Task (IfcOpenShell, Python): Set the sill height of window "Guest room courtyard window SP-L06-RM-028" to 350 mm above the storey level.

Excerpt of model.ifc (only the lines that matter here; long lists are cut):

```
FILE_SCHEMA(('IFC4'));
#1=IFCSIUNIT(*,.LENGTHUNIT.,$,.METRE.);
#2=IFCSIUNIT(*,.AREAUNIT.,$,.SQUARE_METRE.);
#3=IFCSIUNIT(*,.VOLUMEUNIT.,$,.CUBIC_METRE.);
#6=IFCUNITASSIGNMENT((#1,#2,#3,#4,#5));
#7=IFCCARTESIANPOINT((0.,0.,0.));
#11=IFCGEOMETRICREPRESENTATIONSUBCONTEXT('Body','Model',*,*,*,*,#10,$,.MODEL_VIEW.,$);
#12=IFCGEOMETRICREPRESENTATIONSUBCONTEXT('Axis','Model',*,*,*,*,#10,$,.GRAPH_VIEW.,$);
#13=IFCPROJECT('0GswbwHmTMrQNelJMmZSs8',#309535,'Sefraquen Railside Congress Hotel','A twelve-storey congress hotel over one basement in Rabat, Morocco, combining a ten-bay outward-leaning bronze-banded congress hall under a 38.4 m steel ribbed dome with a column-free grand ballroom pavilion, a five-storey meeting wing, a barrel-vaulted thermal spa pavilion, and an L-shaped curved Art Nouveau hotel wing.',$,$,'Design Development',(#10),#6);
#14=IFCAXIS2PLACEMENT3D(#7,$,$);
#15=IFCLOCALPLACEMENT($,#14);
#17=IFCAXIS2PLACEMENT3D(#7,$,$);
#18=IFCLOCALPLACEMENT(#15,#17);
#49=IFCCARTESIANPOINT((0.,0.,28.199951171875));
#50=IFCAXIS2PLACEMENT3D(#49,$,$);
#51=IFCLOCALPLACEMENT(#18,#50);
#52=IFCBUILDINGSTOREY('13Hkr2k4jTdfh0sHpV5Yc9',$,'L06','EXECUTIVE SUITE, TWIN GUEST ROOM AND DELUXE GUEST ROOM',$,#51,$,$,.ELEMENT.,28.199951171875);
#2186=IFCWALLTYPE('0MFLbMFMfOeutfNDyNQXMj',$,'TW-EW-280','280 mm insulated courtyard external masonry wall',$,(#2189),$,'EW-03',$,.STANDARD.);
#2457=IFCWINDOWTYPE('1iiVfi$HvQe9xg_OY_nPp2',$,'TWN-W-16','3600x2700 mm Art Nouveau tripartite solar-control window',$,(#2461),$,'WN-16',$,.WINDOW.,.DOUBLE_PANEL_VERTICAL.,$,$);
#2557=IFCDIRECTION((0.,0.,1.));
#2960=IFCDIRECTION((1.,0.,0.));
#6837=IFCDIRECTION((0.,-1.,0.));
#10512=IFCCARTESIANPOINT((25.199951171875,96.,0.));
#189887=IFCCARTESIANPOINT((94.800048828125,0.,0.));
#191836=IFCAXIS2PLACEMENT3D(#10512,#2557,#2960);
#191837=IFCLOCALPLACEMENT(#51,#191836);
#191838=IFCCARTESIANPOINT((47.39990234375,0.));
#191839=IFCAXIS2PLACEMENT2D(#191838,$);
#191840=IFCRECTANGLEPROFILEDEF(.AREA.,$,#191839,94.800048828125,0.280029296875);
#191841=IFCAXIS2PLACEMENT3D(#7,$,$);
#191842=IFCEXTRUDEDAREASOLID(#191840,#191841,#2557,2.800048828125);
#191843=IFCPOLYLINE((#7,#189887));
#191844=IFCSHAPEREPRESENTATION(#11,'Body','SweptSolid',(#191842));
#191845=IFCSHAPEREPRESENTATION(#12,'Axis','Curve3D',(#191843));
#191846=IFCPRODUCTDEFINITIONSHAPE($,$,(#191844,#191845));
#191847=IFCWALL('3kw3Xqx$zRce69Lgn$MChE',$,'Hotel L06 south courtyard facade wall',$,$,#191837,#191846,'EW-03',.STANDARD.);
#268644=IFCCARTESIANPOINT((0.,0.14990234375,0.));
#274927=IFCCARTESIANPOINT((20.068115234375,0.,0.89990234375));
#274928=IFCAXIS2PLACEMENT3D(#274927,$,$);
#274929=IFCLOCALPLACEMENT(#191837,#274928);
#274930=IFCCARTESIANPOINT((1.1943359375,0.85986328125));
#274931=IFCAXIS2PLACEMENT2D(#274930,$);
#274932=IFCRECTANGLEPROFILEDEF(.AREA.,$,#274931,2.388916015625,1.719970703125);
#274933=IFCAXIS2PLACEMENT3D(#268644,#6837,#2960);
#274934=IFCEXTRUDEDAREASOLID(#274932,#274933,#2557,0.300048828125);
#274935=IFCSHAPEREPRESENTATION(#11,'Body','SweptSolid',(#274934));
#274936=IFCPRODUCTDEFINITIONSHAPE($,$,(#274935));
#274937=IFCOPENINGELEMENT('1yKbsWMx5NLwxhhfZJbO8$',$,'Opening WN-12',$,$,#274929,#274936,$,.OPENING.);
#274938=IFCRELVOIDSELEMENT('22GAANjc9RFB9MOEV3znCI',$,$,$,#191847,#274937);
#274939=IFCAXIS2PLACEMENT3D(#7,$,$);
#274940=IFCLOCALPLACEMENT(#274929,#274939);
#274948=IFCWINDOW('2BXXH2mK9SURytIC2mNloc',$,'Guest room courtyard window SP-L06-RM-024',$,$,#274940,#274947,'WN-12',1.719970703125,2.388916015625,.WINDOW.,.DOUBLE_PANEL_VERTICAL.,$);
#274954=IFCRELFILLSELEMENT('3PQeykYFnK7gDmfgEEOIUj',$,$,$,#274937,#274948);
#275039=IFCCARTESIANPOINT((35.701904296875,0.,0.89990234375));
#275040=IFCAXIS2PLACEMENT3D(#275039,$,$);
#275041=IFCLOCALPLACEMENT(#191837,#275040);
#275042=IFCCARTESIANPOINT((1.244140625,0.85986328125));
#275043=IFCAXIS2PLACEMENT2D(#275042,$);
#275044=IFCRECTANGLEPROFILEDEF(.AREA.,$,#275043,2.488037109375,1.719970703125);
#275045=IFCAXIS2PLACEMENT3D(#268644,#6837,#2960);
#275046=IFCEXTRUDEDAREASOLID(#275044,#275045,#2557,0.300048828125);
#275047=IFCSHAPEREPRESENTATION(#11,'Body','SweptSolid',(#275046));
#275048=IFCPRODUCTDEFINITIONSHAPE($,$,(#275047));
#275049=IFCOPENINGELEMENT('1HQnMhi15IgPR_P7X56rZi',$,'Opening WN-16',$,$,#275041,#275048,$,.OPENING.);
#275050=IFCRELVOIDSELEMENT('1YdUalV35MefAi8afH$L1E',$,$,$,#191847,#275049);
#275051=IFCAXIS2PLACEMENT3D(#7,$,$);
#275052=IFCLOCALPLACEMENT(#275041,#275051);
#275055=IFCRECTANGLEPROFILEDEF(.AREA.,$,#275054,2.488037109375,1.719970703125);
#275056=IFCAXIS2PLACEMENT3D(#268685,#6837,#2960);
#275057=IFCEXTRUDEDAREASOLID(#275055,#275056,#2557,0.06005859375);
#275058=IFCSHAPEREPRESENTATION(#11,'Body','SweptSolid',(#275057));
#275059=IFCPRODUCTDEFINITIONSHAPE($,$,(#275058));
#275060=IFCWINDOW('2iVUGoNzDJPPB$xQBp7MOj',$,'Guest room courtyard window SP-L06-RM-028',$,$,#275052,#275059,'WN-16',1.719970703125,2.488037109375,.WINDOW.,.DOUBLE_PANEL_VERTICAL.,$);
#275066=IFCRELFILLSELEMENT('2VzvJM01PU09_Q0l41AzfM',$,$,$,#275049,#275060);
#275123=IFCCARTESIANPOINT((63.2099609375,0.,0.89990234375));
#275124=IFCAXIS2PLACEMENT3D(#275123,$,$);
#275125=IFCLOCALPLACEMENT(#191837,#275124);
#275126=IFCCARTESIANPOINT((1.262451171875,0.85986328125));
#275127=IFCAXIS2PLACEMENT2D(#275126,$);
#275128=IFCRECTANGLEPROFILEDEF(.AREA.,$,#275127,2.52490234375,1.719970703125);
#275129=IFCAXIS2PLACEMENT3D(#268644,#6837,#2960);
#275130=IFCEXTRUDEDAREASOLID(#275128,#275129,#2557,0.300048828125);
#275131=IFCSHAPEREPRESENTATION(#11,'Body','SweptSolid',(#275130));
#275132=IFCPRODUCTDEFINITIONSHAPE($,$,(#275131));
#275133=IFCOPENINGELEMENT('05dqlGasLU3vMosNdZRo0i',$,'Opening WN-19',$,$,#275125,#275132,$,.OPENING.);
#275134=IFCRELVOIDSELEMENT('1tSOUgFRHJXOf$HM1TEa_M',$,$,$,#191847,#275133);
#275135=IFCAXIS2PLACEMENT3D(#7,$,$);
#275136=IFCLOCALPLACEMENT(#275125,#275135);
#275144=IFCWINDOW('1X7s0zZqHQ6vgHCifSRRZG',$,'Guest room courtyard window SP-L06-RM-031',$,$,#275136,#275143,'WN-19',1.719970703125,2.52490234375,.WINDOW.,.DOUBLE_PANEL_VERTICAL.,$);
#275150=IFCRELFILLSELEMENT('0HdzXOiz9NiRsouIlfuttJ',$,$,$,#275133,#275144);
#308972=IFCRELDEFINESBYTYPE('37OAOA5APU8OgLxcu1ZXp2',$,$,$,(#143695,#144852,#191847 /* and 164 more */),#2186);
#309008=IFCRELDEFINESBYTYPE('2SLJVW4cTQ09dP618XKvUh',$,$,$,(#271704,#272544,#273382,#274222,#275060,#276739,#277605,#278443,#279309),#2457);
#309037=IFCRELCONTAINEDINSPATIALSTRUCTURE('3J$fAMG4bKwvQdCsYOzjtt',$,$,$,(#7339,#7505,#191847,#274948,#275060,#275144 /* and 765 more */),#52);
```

```python
import numpy as np
import ifcopenshell
import ifcopenshell.api.geometry
import ifcopenshell.geom
import ifcopenshell.util.element
import ifcopenshell.util.placement
import ifcopenshell.util.shape
import ifcopenshell.util.unit

model = ifcopenshell.open("model.ifc")
unit_scale = ifcopenshell.util.unit.calculate_unit_scale(model)

window = model.by_id(275060)
opening = window.FillsVoids[0].RelatingOpeningElement
storey = ifcopenshell.util.element.get_container(window, ifc_class="IfcBuildingStorey")
level = ifcopenshell.util.placement.get_local_placement(storey.ObjectPlacement)[2, 3]

# The opening's origin need not be at the sill, so measure its lowest point.
shape = ifcopenshell.geom.create_shape(ifcopenshell.geom.settings(), opening)
bottom = ifcopenshell.util.shape.get_shape_bottom_elevation(shape, shape.geometry) / unit_scale
dz = level + 0.35 / unit_scale - bottom

shift = np.array([0.0, 0.0, dz])
# The window is placed relative to its opening, so it follows when the opening moves.
matrix = ifcopenshell.util.placement.get_local_placement(opening.ObjectPlacement)
matrix[:3, 3] += shift
ifcopenshell.api.geometry.edit_object_placement(
    model, product=opening, matrix=matrix, is_si=False, should_transform_children=True
)

print(f"moved by {dz * unit_scale:+.3f} m")

model.write("model_rev.ifc")
```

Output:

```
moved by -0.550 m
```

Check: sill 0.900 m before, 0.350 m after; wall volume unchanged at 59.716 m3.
